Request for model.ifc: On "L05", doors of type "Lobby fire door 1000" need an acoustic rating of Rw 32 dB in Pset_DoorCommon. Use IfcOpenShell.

First a look at what the model holds.

```python
import ifcopenshell
import ifcopenshell.util.element

model = ifcopenshell.open("model.ifc")
print(model.schema)
storey = next(s for s in model.by_type("IfcBuildingStorey") if s.Name == "L05")
doors = [e for e in ifcopenshell.util.element.get_decomposition(storey) if e.is_a("IfcDoor")]
seen = {}
for e in doors:
    element_type = ifcopenshell.util.element.get_type(e)
    key = (element_type.Name if element_type != e and element_type else None, ifcopenshell.util.element.get_pset(e, "Pset_DoorCommon", "AcousticRating"))
    seen[key] = seen.get(key, 0) + 1
for (name, value), count in sorted(seen.items(), key=str):
    print(count, "x", name, "|", value)
```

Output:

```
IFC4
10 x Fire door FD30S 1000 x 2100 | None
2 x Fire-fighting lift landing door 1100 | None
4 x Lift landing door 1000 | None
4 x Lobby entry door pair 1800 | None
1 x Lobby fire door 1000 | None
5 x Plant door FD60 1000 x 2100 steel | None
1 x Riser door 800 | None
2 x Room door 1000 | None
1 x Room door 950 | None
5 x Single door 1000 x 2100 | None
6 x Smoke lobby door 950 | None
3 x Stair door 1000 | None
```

```python
import ifcopenshell
import ifcopenshell.api.pset
import ifcopenshell.util.element

model = ifcopenshell.open("model.ifc")

storey = next(s for s in model.by_type("IfcBuildingStorey") if s.Name == "L05")
doors = [e for e in ifcopenshell.util.element.get_decomposition(storey) if e.is_a("IfcDoor")]

count = 0
for e in doors:
    element_type = ifcopenshell.util.element.get_type(e)
    if element_type in (None, e) or element_type.Name != "Lobby fire door 1000":
        continue
    # add_pset returns the element's existing set when there is one.
    pset = ifcopenshell.api.pset.add_pset(model, product=e, name="Pset_DoorCommon")
    ifcopenshell.api.pset.edit_pset(model, pset=pset, properties={"AcousticRating": "Rw 32 dB"})
    count += 1

print(count, "doors updated")

model.write("model_edited.ifc")
```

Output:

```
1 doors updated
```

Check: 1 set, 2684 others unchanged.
